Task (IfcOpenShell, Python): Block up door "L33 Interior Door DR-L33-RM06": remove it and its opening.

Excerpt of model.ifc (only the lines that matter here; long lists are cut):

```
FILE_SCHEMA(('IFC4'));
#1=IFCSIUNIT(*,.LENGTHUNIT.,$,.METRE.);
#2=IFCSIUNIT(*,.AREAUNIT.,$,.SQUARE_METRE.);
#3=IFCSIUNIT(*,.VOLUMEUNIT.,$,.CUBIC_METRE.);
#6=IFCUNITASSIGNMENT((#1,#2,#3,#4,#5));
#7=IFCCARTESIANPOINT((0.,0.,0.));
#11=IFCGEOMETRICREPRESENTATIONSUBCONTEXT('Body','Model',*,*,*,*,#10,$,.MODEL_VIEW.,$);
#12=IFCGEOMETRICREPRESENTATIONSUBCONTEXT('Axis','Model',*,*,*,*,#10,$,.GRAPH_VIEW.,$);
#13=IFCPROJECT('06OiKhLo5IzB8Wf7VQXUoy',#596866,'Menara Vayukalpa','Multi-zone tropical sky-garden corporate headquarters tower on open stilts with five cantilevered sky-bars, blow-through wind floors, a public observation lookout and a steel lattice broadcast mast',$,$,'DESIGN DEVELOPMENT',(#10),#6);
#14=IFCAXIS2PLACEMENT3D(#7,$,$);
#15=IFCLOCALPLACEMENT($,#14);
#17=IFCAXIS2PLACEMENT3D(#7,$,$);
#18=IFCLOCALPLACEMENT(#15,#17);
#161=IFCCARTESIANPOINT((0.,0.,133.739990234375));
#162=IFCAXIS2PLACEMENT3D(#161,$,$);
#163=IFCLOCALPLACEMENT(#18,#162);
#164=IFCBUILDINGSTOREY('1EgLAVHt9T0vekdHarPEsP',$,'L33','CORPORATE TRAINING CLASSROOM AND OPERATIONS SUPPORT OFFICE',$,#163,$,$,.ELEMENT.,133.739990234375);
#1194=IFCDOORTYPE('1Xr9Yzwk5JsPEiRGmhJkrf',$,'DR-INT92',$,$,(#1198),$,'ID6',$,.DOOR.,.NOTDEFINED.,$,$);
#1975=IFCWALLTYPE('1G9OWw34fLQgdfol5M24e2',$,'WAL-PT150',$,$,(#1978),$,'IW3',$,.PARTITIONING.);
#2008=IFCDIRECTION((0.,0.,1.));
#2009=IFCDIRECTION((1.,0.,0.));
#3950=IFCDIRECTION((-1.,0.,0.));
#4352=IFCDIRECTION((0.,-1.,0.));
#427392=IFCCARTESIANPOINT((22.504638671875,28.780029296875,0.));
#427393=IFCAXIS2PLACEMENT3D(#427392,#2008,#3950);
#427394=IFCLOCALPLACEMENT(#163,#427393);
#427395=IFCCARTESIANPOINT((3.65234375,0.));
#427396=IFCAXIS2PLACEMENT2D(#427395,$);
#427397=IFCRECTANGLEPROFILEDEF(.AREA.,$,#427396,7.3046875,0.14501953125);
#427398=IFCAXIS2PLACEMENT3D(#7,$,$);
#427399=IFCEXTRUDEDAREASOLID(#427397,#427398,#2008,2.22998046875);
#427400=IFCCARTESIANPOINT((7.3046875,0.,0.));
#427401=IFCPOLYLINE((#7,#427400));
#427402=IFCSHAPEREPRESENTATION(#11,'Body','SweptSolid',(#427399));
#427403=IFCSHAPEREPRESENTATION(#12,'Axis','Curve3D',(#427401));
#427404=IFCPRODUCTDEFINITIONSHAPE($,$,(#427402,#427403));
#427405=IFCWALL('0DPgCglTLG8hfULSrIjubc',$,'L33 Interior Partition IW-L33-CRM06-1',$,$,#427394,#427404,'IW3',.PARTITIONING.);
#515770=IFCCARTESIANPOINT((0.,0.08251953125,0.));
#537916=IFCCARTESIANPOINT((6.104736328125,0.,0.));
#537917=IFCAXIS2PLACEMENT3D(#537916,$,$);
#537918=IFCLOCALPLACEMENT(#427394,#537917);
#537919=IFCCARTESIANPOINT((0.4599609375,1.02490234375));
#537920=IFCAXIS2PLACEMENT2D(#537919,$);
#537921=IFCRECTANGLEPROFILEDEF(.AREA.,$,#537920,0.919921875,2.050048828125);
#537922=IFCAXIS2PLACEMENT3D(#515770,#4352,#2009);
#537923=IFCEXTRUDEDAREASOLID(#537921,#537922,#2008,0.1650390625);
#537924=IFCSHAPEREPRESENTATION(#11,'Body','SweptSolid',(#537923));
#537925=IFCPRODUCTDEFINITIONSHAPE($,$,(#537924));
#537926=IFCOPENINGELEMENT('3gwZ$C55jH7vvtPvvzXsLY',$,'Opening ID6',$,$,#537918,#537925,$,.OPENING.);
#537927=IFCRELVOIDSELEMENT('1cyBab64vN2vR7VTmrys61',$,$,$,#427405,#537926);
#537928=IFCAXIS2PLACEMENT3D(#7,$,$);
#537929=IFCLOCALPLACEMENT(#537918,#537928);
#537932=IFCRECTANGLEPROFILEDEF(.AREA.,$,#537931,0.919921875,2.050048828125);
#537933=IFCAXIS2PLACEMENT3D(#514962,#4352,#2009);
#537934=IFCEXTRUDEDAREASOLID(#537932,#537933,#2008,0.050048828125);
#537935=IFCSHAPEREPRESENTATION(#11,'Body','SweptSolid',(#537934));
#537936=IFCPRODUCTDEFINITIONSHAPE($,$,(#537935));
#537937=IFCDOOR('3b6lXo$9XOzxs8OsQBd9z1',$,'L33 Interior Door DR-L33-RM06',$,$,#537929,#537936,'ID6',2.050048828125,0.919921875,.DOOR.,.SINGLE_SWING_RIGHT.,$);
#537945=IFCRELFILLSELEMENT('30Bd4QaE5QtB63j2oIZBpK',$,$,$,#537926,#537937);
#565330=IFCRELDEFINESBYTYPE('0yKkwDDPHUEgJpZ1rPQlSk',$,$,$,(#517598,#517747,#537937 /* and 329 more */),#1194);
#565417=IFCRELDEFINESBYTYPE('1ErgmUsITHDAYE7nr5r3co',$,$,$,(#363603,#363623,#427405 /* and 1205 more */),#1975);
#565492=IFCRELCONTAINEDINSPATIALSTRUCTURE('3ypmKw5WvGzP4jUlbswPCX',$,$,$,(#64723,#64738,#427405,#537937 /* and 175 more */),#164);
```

```python
import ifcopenshell
import ifcopenshell.api.feature
import ifcopenshell.api.root
import ifcopenshell.geom
import ifcopenshell.util.shape

model = ifcopenshell.open("model.ifc")
settings = ifcopenshell.geom.settings()


def volume(element):
    """Net volume in cubic metres, openings subtracted."""
    shape = ifcopenshell.geom.create_shape(settings, element)
    return ifcopenshell.util.shape.get_volume(shape.geometry)


door = model.by_guid("3b6lXo$9XOzxs8OsQBd9z1")
opening = door.FillsVoids[0].RelatingOpeningElement
wall = opening.VoidsElements[0].RelatingBuildingElement
before = volume(wall)

ifcopenshell.api.root.remove_product(model, product=door)
ifcopenshell.api.feature.remove_feature(model, feature=opening)

after = volume(wall)

print(f"wall volume {before:.3f} -> {after:.3f} m3")

model.write("model_v2.ifc")
```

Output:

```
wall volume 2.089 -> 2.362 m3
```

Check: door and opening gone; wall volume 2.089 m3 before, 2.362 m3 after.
